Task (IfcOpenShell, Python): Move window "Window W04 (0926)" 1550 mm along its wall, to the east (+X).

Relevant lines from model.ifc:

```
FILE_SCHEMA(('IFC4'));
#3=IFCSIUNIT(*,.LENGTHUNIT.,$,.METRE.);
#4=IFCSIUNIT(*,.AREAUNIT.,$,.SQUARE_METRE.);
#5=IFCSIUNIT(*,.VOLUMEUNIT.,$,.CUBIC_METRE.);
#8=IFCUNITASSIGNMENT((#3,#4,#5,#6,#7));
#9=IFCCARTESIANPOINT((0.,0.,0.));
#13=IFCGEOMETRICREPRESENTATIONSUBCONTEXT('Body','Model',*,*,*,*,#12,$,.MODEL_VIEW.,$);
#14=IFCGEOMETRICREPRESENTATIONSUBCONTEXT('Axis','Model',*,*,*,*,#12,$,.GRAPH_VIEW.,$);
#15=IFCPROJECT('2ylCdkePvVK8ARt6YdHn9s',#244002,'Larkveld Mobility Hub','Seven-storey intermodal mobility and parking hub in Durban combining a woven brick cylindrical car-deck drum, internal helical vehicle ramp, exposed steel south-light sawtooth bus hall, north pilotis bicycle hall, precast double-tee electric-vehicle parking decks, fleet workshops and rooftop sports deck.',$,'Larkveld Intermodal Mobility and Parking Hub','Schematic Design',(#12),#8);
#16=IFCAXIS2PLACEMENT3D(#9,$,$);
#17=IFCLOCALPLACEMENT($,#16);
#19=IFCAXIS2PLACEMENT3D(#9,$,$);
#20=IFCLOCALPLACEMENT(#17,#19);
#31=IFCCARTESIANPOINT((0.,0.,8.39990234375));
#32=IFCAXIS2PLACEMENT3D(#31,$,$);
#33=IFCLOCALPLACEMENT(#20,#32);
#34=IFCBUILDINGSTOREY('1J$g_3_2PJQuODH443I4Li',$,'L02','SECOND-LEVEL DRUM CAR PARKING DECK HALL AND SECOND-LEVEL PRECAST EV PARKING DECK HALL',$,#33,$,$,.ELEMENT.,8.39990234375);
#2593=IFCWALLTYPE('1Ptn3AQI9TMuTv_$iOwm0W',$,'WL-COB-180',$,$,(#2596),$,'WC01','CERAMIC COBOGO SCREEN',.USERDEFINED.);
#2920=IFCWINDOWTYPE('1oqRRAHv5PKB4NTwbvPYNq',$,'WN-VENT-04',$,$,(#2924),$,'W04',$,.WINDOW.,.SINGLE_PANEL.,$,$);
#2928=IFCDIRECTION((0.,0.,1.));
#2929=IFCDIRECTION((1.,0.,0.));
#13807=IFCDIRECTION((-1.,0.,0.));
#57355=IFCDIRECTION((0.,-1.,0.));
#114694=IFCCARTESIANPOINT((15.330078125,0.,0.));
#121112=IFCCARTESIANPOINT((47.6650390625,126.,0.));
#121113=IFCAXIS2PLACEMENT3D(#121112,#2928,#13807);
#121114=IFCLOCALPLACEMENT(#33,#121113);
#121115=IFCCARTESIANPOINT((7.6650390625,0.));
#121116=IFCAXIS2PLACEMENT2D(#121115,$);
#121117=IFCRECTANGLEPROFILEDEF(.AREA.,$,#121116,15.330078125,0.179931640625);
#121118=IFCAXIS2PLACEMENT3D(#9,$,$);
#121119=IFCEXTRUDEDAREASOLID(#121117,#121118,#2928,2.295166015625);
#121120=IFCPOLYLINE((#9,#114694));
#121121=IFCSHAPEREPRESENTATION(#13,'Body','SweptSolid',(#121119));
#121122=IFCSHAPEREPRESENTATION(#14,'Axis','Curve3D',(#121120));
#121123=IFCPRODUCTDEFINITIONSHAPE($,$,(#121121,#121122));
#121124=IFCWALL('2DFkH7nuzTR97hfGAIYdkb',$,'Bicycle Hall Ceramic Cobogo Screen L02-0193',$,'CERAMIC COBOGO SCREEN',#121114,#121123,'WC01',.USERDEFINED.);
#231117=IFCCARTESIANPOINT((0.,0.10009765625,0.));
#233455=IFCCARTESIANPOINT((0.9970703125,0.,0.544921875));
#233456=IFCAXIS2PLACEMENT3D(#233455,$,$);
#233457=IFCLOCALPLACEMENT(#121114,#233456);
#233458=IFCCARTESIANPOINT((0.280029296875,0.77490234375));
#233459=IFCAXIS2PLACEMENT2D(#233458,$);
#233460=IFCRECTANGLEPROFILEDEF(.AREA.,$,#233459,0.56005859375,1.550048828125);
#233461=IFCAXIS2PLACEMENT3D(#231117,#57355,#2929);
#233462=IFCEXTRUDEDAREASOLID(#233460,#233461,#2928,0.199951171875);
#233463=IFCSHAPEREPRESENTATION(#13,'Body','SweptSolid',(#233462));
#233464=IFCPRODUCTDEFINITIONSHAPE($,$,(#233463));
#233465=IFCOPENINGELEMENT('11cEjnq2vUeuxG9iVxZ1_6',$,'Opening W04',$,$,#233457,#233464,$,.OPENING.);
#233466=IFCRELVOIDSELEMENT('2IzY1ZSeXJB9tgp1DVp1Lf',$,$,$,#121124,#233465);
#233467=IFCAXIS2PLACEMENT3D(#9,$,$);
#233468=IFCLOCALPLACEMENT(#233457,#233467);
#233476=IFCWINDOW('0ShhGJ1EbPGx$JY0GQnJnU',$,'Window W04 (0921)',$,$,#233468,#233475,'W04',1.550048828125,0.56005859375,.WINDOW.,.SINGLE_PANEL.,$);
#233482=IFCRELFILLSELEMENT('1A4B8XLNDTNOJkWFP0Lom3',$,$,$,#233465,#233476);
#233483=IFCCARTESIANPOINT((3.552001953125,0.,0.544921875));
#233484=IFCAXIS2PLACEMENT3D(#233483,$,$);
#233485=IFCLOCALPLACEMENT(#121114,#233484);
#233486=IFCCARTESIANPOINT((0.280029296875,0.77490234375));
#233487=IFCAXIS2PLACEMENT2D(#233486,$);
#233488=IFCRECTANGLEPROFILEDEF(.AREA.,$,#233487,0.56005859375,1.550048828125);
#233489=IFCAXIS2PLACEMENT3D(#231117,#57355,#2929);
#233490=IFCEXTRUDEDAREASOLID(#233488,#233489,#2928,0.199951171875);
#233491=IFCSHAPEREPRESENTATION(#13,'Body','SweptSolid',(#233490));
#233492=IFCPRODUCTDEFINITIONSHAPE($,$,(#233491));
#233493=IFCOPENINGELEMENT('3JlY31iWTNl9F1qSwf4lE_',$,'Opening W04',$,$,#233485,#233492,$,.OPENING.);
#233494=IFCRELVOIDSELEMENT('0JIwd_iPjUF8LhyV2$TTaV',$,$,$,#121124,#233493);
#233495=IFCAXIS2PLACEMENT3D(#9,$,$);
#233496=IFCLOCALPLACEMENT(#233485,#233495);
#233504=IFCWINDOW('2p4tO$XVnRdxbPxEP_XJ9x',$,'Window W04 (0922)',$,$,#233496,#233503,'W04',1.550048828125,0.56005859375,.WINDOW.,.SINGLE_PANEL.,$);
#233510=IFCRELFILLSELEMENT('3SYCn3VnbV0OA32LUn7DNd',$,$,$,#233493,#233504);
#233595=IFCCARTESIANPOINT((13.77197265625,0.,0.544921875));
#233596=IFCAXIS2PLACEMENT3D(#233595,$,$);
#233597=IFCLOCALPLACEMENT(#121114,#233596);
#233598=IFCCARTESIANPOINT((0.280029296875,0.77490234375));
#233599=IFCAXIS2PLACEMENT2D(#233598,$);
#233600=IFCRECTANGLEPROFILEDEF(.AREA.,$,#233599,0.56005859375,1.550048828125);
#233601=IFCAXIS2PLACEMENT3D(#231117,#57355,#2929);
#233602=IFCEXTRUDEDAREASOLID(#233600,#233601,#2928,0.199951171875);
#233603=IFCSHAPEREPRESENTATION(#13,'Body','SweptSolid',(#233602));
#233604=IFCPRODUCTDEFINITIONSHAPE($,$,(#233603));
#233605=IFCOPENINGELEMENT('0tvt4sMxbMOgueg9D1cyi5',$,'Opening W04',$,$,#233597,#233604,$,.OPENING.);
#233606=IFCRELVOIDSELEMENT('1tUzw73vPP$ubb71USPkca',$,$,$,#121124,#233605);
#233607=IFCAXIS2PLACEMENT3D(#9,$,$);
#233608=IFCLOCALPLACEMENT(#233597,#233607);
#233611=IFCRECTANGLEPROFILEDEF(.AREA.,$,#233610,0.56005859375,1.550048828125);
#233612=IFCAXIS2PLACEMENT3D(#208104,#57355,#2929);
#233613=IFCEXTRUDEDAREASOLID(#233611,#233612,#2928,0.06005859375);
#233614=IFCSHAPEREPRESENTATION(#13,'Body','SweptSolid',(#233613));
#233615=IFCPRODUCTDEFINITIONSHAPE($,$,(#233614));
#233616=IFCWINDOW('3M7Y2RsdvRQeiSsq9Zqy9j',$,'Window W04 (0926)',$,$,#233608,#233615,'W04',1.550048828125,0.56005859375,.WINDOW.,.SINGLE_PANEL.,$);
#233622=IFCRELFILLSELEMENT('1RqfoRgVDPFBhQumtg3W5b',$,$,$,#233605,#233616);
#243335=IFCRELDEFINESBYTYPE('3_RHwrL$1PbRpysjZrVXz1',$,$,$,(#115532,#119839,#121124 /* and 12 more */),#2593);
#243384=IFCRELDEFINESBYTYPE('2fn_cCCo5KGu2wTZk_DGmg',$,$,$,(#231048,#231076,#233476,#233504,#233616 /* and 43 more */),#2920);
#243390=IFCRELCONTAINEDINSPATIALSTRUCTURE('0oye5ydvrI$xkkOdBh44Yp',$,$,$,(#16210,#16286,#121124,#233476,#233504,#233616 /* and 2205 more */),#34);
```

```python
import ifcopenshell
import ifcopenshell.api.geometry
import ifcopenshell.util.placement

model = ifcopenshell.open("model.ifc")

window = model.by_id(233616)
opening = window.FillsVoids[0].RelatingOpeningElement
wall = opening.VoidsElements[0].RelatingBuildingElement

wall_matrix = ifcopenshell.util.placement.get_local_placement(wall.ObjectPlacement)
shift = wall_matrix[:3, 0] * -1.55
before = ifcopenshell.util.placement.get_local_placement(window.ObjectPlacement)[:3, 3].copy()

# The window is placed relative to its opening, so it follows when the opening moves.
matrix = ifcopenshell.util.placement.get_local_placement(opening.ObjectPlacement)
matrix[:3, 3] += shift
ifcopenshell.api.geometry.edit_object_placement(
    model, product=opening, matrix=matrix, is_si=False, should_transform_children=True
)

after = ifcopenshell.util.placement.get_local_placement(window.ObjectPlacement)[:3, 3]
print("window moved by", (after - before).round(3) + 0.0)

model.write("model_rev.ifc")
```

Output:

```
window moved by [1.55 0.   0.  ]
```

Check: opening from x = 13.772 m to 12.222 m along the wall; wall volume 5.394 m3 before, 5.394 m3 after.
